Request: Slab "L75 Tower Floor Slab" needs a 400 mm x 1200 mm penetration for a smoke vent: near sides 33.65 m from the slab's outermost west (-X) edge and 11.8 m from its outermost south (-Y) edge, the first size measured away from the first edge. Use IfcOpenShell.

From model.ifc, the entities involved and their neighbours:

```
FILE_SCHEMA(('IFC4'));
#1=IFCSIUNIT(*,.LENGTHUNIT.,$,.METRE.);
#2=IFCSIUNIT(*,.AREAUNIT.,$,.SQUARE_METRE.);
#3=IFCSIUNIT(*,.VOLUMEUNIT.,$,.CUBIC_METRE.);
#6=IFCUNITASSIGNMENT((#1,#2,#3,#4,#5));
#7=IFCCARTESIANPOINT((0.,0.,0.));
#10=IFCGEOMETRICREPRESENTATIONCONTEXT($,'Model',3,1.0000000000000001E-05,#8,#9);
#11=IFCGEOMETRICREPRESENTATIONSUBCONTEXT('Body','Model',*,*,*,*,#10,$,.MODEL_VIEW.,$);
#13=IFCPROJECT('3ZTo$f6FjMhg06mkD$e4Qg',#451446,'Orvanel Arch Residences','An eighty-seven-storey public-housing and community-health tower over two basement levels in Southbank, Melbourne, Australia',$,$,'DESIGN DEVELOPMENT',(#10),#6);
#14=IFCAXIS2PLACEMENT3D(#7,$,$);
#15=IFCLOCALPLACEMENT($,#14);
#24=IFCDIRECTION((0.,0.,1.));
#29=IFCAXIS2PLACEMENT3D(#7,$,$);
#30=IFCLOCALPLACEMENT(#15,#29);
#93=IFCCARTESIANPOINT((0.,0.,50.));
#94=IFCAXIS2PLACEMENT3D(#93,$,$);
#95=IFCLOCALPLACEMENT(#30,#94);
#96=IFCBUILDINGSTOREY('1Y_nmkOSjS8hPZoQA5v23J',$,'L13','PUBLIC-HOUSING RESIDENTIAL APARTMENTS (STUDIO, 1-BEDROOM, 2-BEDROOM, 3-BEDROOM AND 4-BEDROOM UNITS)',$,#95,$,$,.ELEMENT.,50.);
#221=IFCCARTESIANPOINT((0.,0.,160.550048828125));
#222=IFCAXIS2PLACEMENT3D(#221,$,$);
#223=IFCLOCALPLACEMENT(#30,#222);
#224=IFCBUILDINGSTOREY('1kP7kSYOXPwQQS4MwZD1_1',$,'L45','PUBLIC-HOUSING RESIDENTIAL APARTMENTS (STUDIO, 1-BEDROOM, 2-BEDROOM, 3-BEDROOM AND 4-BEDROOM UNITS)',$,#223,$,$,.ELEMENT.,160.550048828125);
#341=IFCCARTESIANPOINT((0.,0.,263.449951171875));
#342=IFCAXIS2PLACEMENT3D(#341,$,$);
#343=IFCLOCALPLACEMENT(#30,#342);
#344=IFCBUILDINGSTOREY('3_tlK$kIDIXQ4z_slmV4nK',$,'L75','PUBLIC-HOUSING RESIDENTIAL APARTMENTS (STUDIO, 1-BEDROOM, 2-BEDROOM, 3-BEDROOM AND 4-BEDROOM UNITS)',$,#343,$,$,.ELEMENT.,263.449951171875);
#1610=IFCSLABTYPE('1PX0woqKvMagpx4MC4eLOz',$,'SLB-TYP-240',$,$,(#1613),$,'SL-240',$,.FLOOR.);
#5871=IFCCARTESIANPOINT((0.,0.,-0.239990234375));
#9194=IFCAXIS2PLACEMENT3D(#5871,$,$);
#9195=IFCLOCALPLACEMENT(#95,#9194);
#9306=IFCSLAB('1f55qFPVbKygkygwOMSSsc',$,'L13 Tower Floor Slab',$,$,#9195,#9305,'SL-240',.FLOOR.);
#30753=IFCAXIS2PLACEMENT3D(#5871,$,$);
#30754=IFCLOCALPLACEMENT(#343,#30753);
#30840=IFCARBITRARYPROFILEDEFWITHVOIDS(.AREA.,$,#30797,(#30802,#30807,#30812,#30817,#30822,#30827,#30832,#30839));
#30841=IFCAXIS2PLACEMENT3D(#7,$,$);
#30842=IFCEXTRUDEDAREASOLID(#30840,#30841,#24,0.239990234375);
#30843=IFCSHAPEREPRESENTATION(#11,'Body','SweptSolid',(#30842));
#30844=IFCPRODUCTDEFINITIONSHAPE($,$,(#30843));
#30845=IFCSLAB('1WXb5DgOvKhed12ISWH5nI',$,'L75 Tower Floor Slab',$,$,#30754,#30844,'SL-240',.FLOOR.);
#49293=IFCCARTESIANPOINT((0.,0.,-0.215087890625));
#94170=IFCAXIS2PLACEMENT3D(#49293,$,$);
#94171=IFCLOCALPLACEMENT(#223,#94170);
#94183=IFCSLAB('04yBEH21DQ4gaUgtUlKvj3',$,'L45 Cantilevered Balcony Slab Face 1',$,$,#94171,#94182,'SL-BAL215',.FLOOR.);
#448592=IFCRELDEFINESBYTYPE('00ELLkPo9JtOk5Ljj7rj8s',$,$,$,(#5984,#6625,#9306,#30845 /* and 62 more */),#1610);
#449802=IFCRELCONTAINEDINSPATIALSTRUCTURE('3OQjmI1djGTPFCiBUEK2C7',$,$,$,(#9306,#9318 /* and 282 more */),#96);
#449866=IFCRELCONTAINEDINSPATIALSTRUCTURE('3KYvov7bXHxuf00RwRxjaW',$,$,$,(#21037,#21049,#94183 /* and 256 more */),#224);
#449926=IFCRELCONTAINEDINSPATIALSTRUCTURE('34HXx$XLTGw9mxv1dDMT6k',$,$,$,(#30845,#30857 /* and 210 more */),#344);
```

```python
import numpy as np
import ifcopenshell
import ifcopenshell.api.feature
import ifcopenshell.api.geometry
import ifcopenshell.api.root
import ifcopenshell.geom
import ifcopenshell.util.placement
import ifcopenshell.util.representation
import ifcopenshell.util.shape
import ifcopenshell.util.unit

model = ifcopenshell.open("model.ifc")
unit_scale = ifcopenshell.util.unit.calculate_unit_scale(model)
settings = ifcopenshell.geom.settings()


def volume(element):
    """Net volume in cubic metres, openings subtracted."""
    shape = ifcopenshell.geom.create_shape(settings, element)
    return ifcopenshell.util.shape.get_volume(shape.geometry)


slab = model.by_id(30845)
before = volume(slab)

# Extent in the slab's own axes, in metres. The edges named are its -X and -Y sides.
slab_shape = ifcopenshell.geom.create_shape(settings, slab)
vertices = ifcopenshell.util.shape.get_vertices(slab_shape.geometry)
x_min, y_min, bottom = vertices.min(axis=0)
top = vertices[:, 2].max()

opening = ifcopenshell.api.root.create_entity(model, ifc_class="IfcOpeningElement", name="Smoke vent opening", predefined_type="OPENING")
context = ifcopenshell.util.representation.get_context(model, "Model", "Body", "MODEL_VIEW")
width, depth = 0.4, 1.2
outline = [(0.0, 0.0), (width, 0.0), (width, depth), (0.0, depth), (0.0, 0.0)]
# Overshoot both faces by 50 mm so the cut is clean.
shape = ifcopenshell.api.geometry.add_slab_representation(
    model, context=context, depth=top - bottom + 0.1, polyline=outline
)
ifcopenshell.api.geometry.assign_representation(model, product=opening, representation=shape)

matrix = ifcopenshell.util.placement.get_local_placement(slab.ObjectPlacement)
matrix[:, 3] = matrix @ np.append(np.array([x_min + 33.65, y_min + 11.8, bottom - 0.05]) / unit_scale, 1.0)
ifcopenshell.api.geometry.edit_object_placement(model, product=opening, matrix=matrix, is_si=False)
ifcopenshell.api.feature.add_feature(model, feature=opening, element=slab)

after = volume(slab)

print(f"slab volume {before:.3f} -> {after:.3f} m3")

model.write("model-out.ifc")
```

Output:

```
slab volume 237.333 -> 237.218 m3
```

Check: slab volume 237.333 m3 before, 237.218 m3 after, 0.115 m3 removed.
